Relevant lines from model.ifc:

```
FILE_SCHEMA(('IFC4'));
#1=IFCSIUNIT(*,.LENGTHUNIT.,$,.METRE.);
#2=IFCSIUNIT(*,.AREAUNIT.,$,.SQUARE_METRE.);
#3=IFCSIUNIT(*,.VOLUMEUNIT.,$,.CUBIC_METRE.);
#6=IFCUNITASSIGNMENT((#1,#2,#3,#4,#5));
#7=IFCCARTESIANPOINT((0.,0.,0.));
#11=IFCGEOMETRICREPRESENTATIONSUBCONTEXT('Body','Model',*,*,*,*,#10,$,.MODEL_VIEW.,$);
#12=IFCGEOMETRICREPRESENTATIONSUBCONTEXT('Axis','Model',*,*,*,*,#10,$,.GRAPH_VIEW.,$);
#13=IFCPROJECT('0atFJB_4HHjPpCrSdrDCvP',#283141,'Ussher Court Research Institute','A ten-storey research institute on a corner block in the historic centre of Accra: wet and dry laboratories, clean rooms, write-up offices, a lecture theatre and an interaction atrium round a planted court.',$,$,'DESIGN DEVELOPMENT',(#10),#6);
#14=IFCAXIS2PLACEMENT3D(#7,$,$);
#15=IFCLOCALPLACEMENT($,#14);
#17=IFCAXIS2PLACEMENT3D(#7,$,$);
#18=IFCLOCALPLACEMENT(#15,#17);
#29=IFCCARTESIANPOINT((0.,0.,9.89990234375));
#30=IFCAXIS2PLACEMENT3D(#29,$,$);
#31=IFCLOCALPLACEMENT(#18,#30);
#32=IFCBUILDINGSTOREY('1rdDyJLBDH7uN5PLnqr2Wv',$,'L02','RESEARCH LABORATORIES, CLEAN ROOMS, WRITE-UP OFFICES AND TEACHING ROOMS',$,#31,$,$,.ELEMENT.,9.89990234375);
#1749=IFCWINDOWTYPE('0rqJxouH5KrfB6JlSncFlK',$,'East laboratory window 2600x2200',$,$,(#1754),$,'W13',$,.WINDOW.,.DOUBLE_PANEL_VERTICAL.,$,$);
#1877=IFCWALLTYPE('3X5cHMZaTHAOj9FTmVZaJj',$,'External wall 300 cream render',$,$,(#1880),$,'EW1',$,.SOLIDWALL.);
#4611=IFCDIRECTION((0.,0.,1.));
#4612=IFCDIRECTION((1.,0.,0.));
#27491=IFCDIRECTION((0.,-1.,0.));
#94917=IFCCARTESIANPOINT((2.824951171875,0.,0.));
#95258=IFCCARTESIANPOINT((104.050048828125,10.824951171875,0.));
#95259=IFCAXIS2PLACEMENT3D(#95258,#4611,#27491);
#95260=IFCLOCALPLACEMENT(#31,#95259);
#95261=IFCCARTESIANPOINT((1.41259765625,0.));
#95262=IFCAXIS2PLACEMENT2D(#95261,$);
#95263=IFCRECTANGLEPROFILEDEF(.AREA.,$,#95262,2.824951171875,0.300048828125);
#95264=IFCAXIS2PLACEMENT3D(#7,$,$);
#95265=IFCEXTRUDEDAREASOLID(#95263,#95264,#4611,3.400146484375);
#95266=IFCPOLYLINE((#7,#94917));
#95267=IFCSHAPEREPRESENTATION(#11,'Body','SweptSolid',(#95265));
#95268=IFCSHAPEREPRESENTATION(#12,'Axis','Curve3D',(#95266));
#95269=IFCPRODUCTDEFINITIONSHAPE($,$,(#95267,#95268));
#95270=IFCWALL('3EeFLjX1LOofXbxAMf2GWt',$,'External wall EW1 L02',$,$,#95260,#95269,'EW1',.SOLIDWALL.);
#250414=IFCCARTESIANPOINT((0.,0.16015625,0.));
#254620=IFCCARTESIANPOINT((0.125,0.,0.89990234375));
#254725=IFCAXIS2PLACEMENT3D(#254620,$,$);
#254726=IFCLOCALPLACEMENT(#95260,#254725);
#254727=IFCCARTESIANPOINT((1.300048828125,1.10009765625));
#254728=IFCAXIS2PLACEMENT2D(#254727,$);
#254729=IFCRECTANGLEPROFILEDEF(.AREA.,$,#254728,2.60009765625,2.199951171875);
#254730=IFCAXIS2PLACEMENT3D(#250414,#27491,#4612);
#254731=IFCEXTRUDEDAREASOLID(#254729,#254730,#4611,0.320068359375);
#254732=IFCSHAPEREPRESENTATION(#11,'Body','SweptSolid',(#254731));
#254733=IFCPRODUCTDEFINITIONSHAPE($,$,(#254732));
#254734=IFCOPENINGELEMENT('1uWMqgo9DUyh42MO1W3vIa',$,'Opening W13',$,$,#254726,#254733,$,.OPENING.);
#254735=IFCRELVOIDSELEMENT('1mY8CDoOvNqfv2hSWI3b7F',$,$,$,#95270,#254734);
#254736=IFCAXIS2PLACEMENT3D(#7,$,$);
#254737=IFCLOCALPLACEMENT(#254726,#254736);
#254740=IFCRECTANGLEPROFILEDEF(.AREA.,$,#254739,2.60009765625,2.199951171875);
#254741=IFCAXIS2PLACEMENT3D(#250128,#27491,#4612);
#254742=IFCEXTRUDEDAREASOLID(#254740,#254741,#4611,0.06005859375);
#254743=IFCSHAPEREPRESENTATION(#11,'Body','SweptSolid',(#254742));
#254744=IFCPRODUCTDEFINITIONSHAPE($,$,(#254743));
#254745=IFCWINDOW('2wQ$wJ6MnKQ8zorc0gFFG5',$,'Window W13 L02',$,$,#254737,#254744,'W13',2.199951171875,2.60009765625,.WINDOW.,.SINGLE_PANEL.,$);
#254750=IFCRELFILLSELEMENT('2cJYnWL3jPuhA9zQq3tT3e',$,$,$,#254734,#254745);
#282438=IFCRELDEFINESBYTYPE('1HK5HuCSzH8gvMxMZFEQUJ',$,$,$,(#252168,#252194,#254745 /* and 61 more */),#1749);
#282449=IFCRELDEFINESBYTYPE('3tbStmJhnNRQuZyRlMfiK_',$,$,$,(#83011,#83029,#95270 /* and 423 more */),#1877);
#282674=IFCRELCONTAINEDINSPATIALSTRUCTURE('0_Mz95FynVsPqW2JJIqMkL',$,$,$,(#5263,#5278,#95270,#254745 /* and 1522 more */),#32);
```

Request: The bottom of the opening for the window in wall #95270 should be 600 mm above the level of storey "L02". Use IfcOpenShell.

```python
import numpy as np
import ifcopenshell
import ifcopenshell.api.geometry
import ifcopenshell.geom
import ifcopenshell.util.element
import ifcopenshell.util.placement
import ifcopenshell.util.shape
import ifcopenshell.util.unit

model = ifcopenshell.open("model.ifc")
unit_scale = ifcopenshell.util.unit.calculate_unit_scale(model)

window = model.by_guid("2wQ$wJ6MnKQ8zorc0gFFG5")
opening = window.FillsVoids[0].RelatingOpeningElement
storey = ifcopenshell.util.element.get_container(window, ifc_class="IfcBuildingStorey")
level = ifcopenshell.util.placement.get_local_placement(storey.ObjectPlacement)[2, 3]

# The opening's origin need not be at the sill, so measure its lowest point.
shape = ifcopenshell.geom.create_shape(ifcopenshell.geom.settings(), opening)
bottom = ifcopenshell.util.shape.get_shape_bottom_elevation(shape, shape.geometry) / unit_scale
dz = level + 0.6 / unit_scale - bottom

shift = np.array([0.0, 0.0, dz])
# The window is placed relative to its opening, so it follows when the opening moves.
matrix = ifcopenshell.util.placement.get_local_placement(opening.ObjectPlacement)
matrix[:3, 3] += shift
ifcopenshell.api.geometry.edit_object_placement(
    model, product=opening, matrix=matrix, is_si=False, should_transform_children=True
)

print(f"moved by {dz * unit_scale:+.3f} m")

model.write("model_v2.ifc")
```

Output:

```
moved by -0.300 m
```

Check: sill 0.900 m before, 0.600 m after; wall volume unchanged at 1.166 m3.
